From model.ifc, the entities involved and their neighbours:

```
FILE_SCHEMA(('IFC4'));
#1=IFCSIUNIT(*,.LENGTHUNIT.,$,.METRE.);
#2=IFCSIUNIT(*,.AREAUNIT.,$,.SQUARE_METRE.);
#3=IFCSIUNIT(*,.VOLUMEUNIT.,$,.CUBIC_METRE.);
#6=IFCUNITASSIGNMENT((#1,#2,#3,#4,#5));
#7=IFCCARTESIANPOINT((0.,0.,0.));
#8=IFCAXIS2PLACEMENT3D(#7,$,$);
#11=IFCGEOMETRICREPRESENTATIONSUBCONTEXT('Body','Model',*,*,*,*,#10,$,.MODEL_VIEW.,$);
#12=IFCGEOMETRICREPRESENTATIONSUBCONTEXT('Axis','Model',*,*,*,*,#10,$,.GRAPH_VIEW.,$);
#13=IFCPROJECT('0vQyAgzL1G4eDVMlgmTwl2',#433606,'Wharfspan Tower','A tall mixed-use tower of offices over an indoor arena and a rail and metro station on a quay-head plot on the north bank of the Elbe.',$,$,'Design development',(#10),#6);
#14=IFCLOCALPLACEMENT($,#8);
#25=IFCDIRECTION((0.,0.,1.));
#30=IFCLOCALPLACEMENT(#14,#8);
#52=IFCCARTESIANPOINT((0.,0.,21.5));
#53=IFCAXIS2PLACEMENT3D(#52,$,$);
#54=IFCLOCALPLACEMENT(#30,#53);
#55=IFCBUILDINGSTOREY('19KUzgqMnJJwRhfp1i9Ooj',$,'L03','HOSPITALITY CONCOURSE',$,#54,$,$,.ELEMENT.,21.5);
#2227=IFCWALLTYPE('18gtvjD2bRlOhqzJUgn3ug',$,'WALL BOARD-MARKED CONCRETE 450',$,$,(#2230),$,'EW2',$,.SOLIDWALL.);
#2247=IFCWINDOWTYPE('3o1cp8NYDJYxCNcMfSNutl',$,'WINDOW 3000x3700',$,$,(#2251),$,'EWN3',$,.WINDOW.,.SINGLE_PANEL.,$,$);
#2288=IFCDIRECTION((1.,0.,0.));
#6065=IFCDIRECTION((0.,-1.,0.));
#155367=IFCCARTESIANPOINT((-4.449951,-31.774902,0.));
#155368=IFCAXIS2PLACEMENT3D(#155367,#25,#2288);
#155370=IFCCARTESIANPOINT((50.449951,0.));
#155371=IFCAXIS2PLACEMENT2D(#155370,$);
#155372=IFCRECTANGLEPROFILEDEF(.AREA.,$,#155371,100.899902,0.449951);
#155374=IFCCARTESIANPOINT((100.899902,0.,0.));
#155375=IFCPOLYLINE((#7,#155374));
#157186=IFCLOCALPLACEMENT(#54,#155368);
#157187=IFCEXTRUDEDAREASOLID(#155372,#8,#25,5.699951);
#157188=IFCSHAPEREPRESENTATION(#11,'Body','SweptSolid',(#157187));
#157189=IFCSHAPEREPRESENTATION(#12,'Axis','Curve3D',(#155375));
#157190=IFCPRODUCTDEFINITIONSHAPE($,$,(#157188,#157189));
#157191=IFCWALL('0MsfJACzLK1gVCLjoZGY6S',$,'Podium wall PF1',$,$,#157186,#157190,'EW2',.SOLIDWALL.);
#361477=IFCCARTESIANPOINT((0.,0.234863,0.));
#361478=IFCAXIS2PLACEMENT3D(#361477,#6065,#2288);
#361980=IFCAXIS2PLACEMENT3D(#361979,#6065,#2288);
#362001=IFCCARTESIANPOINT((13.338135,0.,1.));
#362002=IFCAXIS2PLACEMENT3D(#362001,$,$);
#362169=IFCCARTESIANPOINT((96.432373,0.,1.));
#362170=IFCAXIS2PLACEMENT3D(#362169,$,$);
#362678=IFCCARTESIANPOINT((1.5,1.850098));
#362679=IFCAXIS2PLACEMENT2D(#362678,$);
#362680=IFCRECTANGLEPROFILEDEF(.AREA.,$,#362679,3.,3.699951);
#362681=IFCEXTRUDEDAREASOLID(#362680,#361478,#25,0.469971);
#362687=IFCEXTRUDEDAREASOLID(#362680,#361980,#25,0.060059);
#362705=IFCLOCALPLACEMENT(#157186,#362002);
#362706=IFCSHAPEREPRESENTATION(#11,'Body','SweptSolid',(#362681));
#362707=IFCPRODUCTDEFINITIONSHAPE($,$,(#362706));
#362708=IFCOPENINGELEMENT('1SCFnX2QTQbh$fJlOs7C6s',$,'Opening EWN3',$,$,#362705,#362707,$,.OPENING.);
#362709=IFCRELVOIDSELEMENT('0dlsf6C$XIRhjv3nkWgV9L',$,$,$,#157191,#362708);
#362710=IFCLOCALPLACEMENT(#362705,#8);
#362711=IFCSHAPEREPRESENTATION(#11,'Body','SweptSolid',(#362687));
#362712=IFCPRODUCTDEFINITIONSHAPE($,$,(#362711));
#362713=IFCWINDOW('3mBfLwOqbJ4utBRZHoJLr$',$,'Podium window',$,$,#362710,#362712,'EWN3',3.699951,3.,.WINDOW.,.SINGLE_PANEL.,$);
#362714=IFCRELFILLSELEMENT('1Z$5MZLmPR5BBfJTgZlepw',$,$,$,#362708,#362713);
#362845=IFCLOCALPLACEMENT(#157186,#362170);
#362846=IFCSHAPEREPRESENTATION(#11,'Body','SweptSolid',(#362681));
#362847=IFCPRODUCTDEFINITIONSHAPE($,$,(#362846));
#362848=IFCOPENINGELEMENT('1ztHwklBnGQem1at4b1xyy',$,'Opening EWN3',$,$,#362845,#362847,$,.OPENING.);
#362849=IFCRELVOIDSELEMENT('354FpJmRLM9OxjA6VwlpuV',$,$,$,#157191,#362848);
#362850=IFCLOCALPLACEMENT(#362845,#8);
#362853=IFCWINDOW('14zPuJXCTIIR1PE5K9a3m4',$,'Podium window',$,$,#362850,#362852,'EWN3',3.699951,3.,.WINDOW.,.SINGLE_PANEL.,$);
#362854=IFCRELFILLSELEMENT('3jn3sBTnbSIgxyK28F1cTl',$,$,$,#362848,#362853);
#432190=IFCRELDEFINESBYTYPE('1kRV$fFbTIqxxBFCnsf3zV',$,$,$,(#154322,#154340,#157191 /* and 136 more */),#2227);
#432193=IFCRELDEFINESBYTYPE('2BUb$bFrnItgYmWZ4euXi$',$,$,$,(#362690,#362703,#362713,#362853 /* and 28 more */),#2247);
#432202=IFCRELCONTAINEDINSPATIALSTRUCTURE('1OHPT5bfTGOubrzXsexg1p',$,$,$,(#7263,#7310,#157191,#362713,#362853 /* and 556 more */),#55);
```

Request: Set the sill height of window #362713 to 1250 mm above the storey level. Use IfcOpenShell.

```python
import numpy as np
import ifcopenshell
import ifcopenshell.api.geometry
import ifcopenshell.geom
import ifcopenshell.util.element
import ifcopenshell.util.placement
import ifcopenshell.util.shape
import ifcopenshell.util.unit

model = ifcopenshell.open("model.ifc")
unit_scale = ifcopenshell.util.unit.calculate_unit_scale(model)

window = model.by_guid("3mBfLwOqbJ4utBRZHoJLr$")
opening = window.FillsVoids[0].RelatingOpeningElement
storey = ifcopenshell.util.element.get_container(window, ifc_class="IfcBuildingStorey")
level = ifcopenshell.util.placement.get_local_placement(storey.ObjectPlacement)[2, 3]

# The opening's origin need not be at the sill, so measure its lowest point.
shape = ifcopenshell.geom.create_shape(ifcopenshell.geom.settings(), opening)
bottom = ifcopenshell.util.shape.get_shape_bottom_elevation(shape, shape.geometry) / unit_scale
dz = level + 1.25 - bottom

shift = np.array([0.0, 0.0, dz])
# The window is placed relative to its opening, so it follows when the opening moves.
matrix = ifcopenshell.util.placement.get_local_placement(opening.ObjectPlacement)
matrix[:3, 3] += shift
ifcopenshell.api.geometry.edit_object_placement(
    model, product=opening, matrix=matrix, is_si=False, should_transform_children=True
)

print(f"moved by {dz * unit_scale:+.3f} m")

model.write("model_rev.ifc")
```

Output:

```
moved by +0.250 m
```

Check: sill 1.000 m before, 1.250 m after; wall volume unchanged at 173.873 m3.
